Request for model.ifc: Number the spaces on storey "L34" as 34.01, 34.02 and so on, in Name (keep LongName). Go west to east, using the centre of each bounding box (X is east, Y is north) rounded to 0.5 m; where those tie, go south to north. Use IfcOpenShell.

First a look at what the model holds.

```python
import ifcopenshell
import ifcopenshell.util.element
import ifcopenshell.util.placement

model = ifcopenshell.open("model.ifc")
print(model.schema)
storey = next(s for s in model.by_type("IfcBuildingStorey") if s.Name == "L34")
spaces = [e for e in ifcopenshell.util.element.get_decomposition(storey) if e.is_a("IfcSpace")]
for e in sorted(spaces, key=lambda e: e.id()):
    origin = ifcopenshell.util.placement.get_local_placement(e.ObjectPlacement)[:3, 3]
    print(e.id(), e.Name, e.LongName, origin.round(2) + 0.0, sep=" | ")
```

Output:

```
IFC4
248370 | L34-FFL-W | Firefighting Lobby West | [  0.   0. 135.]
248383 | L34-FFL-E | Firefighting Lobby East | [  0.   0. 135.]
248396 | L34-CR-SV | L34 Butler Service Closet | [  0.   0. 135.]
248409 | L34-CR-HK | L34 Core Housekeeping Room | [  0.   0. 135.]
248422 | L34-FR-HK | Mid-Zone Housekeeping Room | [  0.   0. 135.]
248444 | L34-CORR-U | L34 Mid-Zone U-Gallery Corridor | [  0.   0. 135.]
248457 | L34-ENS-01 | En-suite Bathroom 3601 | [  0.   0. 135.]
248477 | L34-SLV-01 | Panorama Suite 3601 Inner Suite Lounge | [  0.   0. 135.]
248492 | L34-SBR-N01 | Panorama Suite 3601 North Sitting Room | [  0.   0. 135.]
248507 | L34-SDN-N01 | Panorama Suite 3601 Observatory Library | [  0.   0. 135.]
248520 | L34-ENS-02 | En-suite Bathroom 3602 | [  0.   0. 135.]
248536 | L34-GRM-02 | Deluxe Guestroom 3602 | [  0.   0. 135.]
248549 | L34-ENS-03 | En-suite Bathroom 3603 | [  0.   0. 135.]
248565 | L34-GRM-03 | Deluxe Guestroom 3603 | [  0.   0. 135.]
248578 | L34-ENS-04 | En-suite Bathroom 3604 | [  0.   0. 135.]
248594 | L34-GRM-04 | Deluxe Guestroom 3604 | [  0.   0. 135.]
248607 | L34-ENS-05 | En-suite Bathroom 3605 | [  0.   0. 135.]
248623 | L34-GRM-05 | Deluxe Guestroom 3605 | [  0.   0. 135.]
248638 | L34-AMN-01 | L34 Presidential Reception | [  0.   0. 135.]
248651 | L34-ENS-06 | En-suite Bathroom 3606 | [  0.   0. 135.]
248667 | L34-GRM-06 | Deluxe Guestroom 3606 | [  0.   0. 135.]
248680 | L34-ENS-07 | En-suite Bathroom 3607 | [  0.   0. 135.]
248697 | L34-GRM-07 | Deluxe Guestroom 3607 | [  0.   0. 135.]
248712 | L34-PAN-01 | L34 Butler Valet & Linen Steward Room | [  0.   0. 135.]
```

```python
import ifcopenshell
import ifcopenshell.geom
import ifcopenshell.util.element
import ifcopenshell.util.shape

model = ifcopenshell.open("model.ifc")
settings = ifcopenshell.geom.settings()
settings.set("use-world-coords", True)


def centre(element):
    shape = ifcopenshell.geom.create_shape(settings, element)
    return ifcopenshell.util.shape.get_bbox_centroid(shape.geometry)


storey = next(s for s in model.by_type("IfcBuildingStorey") if s.Name == "L34")
spaces = [e for e in ifcopenshell.util.element.get_decomposition(storey) if e.is_a("IfcSpace")]

# Insertion points can sit at a corner or the storey origin, so sort by the geometry (in metres).
centres = {e: centre(e) for e in spaces}
spaces.sort(key=lambda e: (round(centres[e][0] / 0.5), centres[e][1]))

for i, e in enumerate(spaces, start=1):
    number = f"34.{i:02d}"
    e.Name = number
    print(e.id(), number)

model.write("model_updated.ifc")
```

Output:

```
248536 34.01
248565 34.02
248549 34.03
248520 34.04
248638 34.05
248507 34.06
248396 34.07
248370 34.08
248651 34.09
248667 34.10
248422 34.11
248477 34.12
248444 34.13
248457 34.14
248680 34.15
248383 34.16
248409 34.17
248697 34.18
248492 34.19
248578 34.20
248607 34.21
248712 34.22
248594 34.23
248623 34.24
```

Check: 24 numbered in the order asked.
